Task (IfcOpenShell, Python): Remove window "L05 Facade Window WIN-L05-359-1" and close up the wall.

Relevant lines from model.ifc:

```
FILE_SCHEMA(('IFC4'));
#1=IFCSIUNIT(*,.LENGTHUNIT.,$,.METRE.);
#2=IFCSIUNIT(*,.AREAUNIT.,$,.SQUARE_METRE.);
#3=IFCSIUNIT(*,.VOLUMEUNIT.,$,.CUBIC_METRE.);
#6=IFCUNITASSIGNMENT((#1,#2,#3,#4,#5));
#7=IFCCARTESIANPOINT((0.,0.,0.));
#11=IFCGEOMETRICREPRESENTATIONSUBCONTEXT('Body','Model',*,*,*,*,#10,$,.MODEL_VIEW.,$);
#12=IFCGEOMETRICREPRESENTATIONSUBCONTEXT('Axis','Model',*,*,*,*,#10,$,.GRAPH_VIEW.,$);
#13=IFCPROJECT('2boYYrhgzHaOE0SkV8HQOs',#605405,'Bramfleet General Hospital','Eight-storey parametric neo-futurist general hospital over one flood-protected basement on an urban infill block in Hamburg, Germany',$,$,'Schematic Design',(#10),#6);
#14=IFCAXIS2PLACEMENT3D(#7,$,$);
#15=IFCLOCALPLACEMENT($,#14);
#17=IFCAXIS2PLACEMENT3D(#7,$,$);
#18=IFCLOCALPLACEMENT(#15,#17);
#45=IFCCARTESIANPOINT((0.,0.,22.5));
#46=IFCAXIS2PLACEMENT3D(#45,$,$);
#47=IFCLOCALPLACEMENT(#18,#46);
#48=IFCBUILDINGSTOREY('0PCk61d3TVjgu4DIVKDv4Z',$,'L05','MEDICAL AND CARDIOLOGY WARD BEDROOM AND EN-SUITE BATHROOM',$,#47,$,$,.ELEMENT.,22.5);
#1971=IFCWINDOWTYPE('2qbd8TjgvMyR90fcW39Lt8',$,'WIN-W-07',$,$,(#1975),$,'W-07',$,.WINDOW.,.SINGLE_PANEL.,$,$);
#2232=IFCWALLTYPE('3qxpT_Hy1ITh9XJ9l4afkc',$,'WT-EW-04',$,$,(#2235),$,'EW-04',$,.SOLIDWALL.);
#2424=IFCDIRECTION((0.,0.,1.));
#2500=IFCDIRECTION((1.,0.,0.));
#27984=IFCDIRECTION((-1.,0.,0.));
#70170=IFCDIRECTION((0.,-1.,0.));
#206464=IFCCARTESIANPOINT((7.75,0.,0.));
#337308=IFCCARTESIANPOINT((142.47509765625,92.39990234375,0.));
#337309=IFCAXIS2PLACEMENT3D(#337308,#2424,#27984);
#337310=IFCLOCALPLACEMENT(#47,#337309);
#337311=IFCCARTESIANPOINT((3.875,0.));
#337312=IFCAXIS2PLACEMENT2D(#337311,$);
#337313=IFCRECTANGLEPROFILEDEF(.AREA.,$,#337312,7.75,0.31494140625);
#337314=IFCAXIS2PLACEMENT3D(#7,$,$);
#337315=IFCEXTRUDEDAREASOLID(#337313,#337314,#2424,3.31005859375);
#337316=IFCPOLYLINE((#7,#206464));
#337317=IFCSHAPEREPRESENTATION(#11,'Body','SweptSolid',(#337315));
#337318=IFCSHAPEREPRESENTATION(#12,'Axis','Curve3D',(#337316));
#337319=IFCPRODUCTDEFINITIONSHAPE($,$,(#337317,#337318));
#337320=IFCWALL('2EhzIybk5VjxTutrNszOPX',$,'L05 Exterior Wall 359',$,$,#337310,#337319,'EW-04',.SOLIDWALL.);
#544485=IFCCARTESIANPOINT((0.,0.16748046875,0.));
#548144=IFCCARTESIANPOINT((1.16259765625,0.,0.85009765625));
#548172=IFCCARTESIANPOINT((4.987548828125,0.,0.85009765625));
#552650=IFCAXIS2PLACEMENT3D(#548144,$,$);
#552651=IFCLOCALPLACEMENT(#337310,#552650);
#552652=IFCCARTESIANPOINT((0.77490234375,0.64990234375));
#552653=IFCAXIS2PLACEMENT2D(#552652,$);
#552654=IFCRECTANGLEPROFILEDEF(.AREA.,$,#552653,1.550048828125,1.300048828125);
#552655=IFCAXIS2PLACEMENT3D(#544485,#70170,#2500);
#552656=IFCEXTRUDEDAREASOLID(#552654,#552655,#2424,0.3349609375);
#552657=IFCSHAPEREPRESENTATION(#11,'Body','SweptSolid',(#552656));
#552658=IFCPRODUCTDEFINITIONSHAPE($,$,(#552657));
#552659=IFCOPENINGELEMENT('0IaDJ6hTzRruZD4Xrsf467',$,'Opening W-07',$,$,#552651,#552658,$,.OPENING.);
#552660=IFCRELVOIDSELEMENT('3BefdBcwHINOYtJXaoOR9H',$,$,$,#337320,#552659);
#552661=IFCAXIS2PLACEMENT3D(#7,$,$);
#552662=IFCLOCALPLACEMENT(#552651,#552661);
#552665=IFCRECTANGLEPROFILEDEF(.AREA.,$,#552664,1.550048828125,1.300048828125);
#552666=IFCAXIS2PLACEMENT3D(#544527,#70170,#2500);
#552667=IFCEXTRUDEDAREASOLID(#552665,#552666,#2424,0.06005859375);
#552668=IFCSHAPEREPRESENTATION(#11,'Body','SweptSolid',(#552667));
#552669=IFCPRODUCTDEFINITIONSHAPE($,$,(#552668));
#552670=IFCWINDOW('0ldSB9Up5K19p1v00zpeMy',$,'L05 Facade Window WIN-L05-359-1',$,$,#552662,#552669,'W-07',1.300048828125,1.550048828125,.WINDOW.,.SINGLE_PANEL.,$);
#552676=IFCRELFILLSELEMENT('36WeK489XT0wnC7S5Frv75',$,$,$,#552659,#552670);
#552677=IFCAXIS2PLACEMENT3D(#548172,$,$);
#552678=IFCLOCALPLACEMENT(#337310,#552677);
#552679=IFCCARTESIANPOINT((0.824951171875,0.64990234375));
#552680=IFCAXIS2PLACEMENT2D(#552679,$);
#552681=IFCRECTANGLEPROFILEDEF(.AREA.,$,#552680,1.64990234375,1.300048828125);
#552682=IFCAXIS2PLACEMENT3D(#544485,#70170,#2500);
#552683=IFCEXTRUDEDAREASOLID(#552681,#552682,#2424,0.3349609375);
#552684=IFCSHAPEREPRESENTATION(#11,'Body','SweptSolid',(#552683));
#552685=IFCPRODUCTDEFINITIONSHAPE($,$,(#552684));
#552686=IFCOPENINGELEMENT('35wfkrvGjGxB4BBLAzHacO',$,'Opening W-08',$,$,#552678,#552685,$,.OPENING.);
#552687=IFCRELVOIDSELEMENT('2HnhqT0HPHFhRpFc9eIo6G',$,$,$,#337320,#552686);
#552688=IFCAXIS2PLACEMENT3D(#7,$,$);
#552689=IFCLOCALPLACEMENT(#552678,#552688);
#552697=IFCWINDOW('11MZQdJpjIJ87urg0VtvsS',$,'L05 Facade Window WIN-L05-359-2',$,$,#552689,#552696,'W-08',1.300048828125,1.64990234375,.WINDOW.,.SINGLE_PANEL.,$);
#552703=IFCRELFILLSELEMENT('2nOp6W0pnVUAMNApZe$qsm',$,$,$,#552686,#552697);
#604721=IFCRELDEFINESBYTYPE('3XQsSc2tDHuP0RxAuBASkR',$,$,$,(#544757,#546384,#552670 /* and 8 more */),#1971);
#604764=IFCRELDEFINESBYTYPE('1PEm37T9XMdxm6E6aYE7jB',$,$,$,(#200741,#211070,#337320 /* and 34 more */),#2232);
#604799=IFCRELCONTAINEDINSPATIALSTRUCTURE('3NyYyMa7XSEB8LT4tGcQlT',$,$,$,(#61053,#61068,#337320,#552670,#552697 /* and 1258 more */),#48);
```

```python
import ifcopenshell
import ifcopenshell.api.feature
import ifcopenshell.api.root
import ifcopenshell.geom
import ifcopenshell.util.shape

model = ifcopenshell.open("model.ifc")
settings = ifcopenshell.geom.settings()


def volume(element):
    """Net volume in cubic metres, openings subtracted."""
    shape = ifcopenshell.geom.create_shape(settings, element)
    return ifcopenshell.util.shape.get_volume(shape.geometry)


window = model.by_guid("0ldSB9Up5K19p1v00zpeMy")
opening = window.FillsVoids[0].RelatingOpeningElement
wall = opening.VoidsElements[0].RelatingBuildingElement
before = volume(wall)

ifcopenshell.api.root.remove_product(model, product=window)
ifcopenshell.api.feature.remove_feature(model, feature=opening)

after = volume(wall)

print(f"wall volume {before:.3f} -> {after:.3f} m3")

model.write("model_edited.ifc")
```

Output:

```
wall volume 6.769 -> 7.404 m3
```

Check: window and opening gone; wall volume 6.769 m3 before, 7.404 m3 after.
